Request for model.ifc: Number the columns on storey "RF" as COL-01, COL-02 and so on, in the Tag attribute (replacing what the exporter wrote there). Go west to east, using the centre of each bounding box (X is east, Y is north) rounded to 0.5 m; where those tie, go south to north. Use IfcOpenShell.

First a look at what the model holds.

```python
import ifcopenshell
import ifcopenshell.util.element
import ifcopenshell.util.placement

model = ifcopenshell.open("model.ifc")
print(model.schema)
storey = next(s for s in model.by_type("IfcBuildingStorey") if s.Name == "RF")
columns = [e for e in ifcopenshell.util.element.get_decomposition(storey) if e.is_a("IfcColumn")]
for e in sorted(columns, key=lambda e: e.id()):
    origin = ifcopenshell.util.placement.get_local_placement(e.ObjectPlacement)[:3, 3]
    print(e.id(), e.Tag, e.Name, origin.round(2) + 0.0, sep=" | ")
```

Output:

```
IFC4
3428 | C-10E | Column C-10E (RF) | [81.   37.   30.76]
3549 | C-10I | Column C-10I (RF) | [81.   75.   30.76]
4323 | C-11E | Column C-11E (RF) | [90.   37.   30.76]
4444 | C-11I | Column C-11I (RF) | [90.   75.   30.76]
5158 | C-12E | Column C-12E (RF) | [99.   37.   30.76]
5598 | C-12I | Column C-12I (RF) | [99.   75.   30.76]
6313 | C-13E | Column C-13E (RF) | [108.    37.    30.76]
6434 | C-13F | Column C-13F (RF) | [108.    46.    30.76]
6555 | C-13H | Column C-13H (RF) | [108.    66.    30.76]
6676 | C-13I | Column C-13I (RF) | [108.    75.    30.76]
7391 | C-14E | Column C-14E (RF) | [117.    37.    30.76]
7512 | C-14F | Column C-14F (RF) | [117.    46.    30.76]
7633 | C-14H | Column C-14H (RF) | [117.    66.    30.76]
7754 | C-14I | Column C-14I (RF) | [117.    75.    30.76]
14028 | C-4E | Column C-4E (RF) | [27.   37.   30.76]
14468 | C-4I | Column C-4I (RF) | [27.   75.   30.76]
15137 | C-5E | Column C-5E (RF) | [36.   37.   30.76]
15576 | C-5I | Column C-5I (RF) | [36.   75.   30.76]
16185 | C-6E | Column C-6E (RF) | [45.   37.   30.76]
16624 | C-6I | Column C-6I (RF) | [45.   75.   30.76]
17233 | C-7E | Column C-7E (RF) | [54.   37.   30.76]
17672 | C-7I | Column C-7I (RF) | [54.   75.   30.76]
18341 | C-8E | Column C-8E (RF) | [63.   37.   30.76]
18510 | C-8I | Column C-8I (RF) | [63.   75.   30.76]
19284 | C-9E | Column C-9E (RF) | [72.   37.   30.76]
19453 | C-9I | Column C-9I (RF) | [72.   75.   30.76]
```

```python
import ifcopenshell
import ifcopenshell.geom
import ifcopenshell.util.element
import ifcopenshell.util.shape

model = ifcopenshell.open("model.ifc")
settings = ifcopenshell.geom.settings()
settings.set("use-world-coords", True)


def centre(element):
    shape = ifcopenshell.geom.create_shape(settings, element)
    return ifcopenshell.util.shape.get_bbox_centroid(shape.geometry)


storey = next(s for s in model.by_type("IfcBuildingStorey") if s.Name == "RF")
columns = [e for e in ifcopenshell.util.element.get_decomposition(storey) if e.is_a("IfcColumn")]

# Insertion points can sit at a corner or the storey origin, so sort by the geometry (in metres).
centres = {e: centre(e) for e in columns}
columns.sort(key=lambda e: (round(centres[e][0] / 0.5), centres[e][1]))

for i, e in enumerate(columns, start=1):
    number = f"COL-{i:02d}"
    e.Tag = number
    print(e.id(), number)

model.write("model_rev.ifc")
```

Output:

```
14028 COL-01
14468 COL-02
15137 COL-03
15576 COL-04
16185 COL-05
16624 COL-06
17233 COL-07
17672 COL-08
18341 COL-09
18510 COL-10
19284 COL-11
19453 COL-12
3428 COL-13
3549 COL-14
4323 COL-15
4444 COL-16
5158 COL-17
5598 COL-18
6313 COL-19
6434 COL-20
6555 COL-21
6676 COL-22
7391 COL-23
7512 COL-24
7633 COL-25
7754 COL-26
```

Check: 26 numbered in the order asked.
